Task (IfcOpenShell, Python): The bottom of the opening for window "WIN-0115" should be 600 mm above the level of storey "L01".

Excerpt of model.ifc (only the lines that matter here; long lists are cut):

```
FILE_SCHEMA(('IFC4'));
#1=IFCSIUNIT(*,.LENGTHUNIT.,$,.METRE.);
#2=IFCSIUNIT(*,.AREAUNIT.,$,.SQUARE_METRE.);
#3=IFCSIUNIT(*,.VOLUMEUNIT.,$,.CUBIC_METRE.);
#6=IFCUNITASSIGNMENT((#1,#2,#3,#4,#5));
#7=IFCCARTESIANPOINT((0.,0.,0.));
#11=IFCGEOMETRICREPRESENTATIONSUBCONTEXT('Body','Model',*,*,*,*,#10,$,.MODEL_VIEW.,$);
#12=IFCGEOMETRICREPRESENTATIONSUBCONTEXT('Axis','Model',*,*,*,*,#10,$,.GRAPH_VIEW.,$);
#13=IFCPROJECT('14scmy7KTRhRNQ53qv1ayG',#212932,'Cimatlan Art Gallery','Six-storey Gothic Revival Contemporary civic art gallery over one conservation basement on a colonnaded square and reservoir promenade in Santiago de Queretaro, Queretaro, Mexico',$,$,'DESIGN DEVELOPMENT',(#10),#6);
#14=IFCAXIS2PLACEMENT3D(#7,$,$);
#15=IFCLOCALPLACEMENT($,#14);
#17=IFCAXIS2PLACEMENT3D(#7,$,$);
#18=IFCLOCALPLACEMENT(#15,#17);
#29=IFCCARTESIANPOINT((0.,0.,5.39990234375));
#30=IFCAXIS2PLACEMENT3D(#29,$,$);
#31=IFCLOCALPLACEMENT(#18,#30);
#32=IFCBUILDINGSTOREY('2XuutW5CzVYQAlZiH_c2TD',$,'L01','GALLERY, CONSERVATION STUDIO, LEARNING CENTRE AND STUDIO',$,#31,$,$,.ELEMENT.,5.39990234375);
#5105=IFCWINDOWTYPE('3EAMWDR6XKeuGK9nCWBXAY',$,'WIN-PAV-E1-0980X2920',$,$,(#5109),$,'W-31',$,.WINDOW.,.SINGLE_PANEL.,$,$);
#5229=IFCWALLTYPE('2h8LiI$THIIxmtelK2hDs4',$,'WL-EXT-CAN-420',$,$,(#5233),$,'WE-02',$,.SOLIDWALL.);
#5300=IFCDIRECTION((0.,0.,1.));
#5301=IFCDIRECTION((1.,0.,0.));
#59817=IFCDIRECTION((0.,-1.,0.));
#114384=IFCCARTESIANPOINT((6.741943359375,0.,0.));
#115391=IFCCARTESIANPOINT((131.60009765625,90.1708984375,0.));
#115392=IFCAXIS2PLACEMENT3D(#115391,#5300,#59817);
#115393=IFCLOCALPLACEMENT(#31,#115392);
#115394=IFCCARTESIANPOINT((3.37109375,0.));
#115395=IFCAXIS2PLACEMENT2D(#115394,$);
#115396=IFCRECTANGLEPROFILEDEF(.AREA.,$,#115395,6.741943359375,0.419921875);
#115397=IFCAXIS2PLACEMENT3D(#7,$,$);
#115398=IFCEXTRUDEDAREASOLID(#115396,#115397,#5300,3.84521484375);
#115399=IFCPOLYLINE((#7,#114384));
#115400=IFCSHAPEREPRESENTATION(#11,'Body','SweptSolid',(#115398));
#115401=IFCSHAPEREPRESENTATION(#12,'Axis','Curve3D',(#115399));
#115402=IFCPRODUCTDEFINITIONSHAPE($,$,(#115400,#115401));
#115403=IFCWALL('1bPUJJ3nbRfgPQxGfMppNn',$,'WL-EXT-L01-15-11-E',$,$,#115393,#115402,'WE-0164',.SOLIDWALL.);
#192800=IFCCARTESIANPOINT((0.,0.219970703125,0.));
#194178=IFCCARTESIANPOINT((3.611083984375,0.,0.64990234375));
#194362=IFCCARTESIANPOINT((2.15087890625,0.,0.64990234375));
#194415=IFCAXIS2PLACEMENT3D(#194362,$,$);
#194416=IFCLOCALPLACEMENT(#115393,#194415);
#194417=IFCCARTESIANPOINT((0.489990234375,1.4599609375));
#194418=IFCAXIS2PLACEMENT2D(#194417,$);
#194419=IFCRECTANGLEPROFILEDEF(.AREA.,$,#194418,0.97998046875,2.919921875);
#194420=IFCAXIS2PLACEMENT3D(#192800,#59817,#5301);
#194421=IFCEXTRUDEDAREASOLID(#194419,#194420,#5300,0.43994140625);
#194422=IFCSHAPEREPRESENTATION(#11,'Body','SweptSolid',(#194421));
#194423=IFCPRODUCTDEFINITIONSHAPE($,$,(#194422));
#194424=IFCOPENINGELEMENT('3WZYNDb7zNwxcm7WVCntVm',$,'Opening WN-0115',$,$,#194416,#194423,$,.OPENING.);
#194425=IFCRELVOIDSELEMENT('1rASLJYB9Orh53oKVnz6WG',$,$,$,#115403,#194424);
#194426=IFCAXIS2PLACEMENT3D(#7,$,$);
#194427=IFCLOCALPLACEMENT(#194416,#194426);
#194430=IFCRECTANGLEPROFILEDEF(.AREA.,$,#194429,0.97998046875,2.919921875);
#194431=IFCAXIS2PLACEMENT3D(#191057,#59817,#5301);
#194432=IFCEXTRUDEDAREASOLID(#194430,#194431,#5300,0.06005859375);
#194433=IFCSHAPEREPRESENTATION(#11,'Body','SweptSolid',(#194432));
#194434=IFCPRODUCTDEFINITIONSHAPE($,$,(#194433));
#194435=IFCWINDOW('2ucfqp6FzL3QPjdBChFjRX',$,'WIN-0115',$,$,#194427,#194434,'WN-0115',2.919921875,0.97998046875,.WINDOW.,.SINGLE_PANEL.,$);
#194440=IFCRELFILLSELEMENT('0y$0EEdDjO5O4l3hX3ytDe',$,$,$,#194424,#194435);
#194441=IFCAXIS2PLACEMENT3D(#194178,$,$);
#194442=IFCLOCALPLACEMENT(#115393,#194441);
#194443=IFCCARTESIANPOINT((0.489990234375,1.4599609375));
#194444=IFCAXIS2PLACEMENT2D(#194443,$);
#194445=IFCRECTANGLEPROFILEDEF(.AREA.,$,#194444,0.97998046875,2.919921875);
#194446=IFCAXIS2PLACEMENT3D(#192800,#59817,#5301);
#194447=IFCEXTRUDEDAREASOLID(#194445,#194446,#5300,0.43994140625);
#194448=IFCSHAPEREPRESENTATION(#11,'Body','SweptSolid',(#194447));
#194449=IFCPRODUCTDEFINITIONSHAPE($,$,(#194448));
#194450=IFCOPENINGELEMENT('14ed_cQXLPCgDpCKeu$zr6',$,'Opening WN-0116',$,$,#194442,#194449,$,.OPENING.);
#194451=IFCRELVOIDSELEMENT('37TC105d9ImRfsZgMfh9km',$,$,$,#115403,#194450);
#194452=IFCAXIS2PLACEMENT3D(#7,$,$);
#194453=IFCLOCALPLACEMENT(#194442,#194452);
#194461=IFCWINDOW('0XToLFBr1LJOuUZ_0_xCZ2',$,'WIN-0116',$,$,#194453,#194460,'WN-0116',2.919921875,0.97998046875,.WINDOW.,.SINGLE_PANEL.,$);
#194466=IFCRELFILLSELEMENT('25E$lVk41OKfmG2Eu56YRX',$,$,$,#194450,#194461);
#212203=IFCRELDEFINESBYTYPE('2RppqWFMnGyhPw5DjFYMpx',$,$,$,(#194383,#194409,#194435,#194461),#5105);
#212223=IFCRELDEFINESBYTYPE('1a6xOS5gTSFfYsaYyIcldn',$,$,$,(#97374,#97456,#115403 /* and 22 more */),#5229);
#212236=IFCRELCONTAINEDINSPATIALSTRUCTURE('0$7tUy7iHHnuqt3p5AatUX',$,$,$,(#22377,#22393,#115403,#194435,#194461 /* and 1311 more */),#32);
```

```python
import numpy as np
import ifcopenshell
import ifcopenshell.api.geometry
import ifcopenshell.geom
import ifcopenshell.util.element
import ifcopenshell.util.placement
import ifcopenshell.util.shape
import ifcopenshell.util.unit

model = ifcopenshell.open("model.ifc")
unit_scale = ifcopenshell.util.unit.calculate_unit_scale(model)

window = model.by_guid("2ucfqp6FzL3QPjdBChFjRX")
opening = window.FillsVoids[0].RelatingOpeningElement
storey = ifcopenshell.util.element.get_container(window, ifc_class="IfcBuildingStorey")
level = ifcopenshell.util.placement.get_local_placement(storey.ObjectPlacement)[2, 3]

# The opening's origin need not be at the sill, so measure its lowest point.
shape = ifcopenshell.geom.create_shape(ifcopenshell.geom.settings(), opening)
bottom = ifcopenshell.util.shape.get_shape_bottom_elevation(shape, shape.geometry) / unit_scale
dz = level + 0.6 / unit_scale - bottom

shift = np.array([0.0, 0.0, dz])
# The window is placed relative to its opening, so it follows when the opening moves.
matrix = ifcopenshell.util.placement.get_local_placement(opening.ObjectPlacement)
matrix[:3, 3] += shift
ifcopenshell.api.geometry.edit_object_placement(
    model, product=opening, matrix=matrix, is_si=False, should_transform_children=True
)

print(f"moved by {dz * unit_scale:+.3f} m")

model.write("model_updated.ifc")
```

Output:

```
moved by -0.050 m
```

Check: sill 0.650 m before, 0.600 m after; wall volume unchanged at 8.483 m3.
